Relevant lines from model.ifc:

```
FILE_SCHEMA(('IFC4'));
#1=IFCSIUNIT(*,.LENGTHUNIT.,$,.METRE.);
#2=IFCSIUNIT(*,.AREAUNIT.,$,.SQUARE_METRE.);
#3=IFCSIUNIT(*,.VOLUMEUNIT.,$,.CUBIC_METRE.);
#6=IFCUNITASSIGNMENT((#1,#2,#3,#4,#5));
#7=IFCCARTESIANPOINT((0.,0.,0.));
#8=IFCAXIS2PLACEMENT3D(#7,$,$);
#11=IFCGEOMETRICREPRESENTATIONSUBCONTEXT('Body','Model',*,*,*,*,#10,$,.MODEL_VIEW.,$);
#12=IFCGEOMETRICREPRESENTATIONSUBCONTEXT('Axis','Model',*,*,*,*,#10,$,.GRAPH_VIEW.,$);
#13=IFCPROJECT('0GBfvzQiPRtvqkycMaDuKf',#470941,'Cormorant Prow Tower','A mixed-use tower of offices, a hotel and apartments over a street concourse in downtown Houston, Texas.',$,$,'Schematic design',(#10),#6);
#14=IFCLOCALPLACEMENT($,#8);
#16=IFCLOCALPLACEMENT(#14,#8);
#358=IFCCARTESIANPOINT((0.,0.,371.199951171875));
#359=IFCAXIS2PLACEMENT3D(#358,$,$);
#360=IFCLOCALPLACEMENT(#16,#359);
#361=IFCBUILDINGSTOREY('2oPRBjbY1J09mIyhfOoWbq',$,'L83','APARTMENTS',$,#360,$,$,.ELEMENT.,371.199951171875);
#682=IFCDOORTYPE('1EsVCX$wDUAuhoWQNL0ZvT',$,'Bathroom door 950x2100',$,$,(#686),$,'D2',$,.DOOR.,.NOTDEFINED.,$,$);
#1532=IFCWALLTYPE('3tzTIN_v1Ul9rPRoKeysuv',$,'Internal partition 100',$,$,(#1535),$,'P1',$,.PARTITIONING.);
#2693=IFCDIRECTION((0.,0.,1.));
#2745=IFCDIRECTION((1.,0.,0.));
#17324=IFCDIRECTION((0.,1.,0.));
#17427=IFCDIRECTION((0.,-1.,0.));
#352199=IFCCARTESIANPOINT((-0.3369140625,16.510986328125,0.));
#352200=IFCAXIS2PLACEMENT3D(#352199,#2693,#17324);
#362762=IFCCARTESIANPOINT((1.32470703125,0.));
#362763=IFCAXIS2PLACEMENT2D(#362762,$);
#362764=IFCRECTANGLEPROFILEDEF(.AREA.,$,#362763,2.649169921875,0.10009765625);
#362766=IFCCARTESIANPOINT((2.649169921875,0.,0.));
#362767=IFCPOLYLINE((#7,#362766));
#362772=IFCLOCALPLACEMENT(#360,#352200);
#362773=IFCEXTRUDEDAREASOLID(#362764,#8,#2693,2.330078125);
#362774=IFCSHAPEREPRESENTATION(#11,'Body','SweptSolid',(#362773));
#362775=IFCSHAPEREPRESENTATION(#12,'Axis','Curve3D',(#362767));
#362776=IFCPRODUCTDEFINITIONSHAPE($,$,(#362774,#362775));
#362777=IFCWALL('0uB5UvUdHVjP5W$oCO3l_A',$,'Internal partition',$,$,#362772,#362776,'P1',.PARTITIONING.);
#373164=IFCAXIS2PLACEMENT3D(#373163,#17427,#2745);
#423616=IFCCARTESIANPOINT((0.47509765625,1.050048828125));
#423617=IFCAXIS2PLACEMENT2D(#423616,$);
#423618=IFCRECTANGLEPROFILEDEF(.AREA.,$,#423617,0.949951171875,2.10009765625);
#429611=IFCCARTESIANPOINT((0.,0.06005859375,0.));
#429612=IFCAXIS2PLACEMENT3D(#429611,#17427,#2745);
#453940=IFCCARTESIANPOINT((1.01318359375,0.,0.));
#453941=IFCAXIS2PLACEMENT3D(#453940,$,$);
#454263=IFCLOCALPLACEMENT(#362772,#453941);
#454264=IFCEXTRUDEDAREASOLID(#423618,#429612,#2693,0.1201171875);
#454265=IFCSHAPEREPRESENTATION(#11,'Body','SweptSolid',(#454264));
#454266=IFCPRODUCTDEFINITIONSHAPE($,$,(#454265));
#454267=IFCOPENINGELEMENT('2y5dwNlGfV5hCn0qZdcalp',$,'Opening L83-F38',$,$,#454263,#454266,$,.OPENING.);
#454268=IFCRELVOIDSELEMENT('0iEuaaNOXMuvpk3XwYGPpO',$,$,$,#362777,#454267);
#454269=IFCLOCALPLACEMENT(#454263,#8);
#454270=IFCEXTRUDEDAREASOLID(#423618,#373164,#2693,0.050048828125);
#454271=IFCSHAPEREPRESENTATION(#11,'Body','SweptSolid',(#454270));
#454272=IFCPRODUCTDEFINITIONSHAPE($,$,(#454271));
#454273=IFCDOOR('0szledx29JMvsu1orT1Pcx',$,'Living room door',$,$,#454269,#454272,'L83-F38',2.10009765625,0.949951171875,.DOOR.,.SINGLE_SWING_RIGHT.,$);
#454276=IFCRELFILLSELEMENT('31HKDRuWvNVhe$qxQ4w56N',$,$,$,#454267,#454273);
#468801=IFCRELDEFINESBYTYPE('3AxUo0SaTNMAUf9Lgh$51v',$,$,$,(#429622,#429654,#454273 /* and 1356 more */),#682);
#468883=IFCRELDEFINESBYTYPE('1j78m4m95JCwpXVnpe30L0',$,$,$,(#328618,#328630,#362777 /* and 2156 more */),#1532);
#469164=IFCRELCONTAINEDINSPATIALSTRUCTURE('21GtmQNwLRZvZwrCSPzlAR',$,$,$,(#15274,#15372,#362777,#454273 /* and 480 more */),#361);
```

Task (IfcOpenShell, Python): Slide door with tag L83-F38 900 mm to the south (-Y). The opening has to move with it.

```python
import ifcopenshell
import ifcopenshell.api.geometry
import ifcopenshell.util.placement

model = ifcopenshell.open("model.ifc")

door = model.by_guid("0szledx29JMvsu1orT1Pcx")
opening = door.FillsVoids[0].RelatingOpeningElement
wall = opening.VoidsElements[0].RelatingBuildingElement

wall_matrix = ifcopenshell.util.placement.get_local_placement(wall.ObjectPlacement)
shift = wall_matrix[:3, 0] * -0.9
before = ifcopenshell.util.placement.get_local_placement(door.ObjectPlacement)[:3, 3].copy()

# The door is placed relative to its opening, so it follows when the opening moves.
matrix = ifcopenshell.util.placement.get_local_placement(opening.ObjectPlacement)
matrix[:3, 3] += shift
ifcopenshell.api.geometry.edit_object_placement(
    model, product=opening, matrix=matrix, is_si=False, should_transform_children=True
)

after = ifcopenshell.util.placement.get_local_placement(door.ObjectPlacement)[:3, 3]
print("door moved by", (after - before).round(3) + 0.0)

model.write("model_edited.ifc")
```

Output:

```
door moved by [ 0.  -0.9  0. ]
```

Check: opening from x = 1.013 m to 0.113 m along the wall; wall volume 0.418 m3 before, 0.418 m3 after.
